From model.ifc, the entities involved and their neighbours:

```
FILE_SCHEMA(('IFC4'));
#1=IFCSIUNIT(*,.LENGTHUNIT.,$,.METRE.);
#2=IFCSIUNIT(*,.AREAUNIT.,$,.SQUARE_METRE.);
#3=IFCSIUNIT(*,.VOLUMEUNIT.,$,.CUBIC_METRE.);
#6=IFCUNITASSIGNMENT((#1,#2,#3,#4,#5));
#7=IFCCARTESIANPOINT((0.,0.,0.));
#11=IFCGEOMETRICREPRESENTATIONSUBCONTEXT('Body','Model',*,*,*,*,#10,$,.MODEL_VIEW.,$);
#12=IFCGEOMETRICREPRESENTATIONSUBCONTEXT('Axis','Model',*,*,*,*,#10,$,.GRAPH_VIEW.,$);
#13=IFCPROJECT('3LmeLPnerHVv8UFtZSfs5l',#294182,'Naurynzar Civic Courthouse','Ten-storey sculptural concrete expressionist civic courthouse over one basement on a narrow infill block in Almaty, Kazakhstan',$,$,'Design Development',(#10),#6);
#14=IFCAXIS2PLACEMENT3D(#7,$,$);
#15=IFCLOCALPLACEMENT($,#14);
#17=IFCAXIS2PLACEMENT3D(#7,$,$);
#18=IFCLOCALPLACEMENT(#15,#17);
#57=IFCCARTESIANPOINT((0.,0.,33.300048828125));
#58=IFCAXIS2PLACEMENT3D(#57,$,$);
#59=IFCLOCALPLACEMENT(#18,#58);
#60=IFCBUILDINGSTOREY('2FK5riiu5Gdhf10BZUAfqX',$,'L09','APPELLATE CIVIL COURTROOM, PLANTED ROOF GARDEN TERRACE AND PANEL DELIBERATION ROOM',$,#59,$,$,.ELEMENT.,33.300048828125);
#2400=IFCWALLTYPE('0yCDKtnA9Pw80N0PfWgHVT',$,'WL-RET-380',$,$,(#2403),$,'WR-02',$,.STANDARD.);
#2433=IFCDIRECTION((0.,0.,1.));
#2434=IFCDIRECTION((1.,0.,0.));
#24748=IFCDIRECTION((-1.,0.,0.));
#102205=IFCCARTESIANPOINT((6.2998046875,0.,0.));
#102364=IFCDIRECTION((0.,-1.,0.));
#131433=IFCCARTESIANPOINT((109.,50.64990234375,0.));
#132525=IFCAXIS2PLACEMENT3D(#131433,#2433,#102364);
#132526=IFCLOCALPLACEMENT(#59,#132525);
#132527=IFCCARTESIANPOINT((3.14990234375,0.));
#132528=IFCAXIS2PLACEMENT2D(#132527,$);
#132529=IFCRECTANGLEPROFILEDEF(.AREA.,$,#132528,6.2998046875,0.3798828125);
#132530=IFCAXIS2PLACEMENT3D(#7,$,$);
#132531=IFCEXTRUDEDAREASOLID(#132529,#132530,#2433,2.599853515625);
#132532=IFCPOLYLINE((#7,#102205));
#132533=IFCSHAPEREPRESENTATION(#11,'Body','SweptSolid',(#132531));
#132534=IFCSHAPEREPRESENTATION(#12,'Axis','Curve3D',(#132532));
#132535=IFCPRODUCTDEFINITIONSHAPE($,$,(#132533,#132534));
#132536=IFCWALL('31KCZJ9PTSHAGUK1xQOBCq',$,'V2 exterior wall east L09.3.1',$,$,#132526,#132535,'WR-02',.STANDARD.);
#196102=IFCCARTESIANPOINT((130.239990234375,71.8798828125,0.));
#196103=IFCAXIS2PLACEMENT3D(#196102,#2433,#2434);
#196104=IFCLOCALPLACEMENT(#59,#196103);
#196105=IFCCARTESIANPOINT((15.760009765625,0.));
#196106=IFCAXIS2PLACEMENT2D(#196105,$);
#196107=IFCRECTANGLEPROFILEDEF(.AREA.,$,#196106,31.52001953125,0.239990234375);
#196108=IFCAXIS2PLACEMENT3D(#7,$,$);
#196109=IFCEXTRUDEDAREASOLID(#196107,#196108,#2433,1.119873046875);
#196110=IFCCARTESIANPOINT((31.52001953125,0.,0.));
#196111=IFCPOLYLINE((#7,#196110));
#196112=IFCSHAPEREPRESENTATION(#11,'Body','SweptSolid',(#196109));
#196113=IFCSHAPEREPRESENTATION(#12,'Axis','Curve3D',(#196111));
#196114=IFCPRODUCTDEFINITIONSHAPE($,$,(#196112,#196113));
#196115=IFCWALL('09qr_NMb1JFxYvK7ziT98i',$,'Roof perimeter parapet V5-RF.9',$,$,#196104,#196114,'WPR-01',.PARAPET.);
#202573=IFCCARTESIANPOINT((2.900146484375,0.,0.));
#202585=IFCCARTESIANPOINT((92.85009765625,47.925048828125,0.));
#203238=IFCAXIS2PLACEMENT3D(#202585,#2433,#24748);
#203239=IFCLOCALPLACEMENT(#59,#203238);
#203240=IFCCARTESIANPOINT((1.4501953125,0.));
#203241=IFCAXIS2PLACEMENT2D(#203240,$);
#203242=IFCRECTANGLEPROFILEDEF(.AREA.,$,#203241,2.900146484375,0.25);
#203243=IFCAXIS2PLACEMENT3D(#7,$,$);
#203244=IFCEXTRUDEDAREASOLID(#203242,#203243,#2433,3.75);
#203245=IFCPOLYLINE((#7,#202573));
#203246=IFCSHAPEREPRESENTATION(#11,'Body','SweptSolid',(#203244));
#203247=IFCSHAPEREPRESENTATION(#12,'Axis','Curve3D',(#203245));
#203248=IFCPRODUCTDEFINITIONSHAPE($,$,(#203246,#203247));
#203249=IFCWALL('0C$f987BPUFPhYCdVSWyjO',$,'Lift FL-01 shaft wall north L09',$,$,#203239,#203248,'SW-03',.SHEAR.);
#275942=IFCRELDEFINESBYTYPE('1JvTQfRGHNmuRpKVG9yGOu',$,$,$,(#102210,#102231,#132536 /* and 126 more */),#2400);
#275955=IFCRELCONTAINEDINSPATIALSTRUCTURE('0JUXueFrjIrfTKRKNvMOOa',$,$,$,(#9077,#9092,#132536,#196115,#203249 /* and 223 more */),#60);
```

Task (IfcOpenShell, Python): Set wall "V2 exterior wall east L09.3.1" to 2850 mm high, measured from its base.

```python
import ifcopenshell
import ifcopenshell.geom
import ifcopenshell.util.representation
import ifcopenshell.util.shape

model = ifcopenshell.open("model.ifc")
settings = ifcopenshell.geom.settings()


def volume(element):
    """Net volume in cubic metres, openings subtracted."""
    shape = ifcopenshell.geom.create_shape(settings, element)
    return ifcopenshell.util.shape.get_volume(shape.geometry)


wall = model.by_guid("31KCZJ9PTSHAGUK1xQOBCq")
before = volume(wall)

body = ifcopenshell.util.representation.get_representation(wall, "Model", "Body")
solid = body.Items[0]
old_height = solid.Depth
solid.Depth = 2.85
after = volume(wall)

print(f"height {old_height:g} -> {solid.Depth:g}, volume {before:.3f} -> {after:.3f} m3")

model.write("model_v2.ifc")
```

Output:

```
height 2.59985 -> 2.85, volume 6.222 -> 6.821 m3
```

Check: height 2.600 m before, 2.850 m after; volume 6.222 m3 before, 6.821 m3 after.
